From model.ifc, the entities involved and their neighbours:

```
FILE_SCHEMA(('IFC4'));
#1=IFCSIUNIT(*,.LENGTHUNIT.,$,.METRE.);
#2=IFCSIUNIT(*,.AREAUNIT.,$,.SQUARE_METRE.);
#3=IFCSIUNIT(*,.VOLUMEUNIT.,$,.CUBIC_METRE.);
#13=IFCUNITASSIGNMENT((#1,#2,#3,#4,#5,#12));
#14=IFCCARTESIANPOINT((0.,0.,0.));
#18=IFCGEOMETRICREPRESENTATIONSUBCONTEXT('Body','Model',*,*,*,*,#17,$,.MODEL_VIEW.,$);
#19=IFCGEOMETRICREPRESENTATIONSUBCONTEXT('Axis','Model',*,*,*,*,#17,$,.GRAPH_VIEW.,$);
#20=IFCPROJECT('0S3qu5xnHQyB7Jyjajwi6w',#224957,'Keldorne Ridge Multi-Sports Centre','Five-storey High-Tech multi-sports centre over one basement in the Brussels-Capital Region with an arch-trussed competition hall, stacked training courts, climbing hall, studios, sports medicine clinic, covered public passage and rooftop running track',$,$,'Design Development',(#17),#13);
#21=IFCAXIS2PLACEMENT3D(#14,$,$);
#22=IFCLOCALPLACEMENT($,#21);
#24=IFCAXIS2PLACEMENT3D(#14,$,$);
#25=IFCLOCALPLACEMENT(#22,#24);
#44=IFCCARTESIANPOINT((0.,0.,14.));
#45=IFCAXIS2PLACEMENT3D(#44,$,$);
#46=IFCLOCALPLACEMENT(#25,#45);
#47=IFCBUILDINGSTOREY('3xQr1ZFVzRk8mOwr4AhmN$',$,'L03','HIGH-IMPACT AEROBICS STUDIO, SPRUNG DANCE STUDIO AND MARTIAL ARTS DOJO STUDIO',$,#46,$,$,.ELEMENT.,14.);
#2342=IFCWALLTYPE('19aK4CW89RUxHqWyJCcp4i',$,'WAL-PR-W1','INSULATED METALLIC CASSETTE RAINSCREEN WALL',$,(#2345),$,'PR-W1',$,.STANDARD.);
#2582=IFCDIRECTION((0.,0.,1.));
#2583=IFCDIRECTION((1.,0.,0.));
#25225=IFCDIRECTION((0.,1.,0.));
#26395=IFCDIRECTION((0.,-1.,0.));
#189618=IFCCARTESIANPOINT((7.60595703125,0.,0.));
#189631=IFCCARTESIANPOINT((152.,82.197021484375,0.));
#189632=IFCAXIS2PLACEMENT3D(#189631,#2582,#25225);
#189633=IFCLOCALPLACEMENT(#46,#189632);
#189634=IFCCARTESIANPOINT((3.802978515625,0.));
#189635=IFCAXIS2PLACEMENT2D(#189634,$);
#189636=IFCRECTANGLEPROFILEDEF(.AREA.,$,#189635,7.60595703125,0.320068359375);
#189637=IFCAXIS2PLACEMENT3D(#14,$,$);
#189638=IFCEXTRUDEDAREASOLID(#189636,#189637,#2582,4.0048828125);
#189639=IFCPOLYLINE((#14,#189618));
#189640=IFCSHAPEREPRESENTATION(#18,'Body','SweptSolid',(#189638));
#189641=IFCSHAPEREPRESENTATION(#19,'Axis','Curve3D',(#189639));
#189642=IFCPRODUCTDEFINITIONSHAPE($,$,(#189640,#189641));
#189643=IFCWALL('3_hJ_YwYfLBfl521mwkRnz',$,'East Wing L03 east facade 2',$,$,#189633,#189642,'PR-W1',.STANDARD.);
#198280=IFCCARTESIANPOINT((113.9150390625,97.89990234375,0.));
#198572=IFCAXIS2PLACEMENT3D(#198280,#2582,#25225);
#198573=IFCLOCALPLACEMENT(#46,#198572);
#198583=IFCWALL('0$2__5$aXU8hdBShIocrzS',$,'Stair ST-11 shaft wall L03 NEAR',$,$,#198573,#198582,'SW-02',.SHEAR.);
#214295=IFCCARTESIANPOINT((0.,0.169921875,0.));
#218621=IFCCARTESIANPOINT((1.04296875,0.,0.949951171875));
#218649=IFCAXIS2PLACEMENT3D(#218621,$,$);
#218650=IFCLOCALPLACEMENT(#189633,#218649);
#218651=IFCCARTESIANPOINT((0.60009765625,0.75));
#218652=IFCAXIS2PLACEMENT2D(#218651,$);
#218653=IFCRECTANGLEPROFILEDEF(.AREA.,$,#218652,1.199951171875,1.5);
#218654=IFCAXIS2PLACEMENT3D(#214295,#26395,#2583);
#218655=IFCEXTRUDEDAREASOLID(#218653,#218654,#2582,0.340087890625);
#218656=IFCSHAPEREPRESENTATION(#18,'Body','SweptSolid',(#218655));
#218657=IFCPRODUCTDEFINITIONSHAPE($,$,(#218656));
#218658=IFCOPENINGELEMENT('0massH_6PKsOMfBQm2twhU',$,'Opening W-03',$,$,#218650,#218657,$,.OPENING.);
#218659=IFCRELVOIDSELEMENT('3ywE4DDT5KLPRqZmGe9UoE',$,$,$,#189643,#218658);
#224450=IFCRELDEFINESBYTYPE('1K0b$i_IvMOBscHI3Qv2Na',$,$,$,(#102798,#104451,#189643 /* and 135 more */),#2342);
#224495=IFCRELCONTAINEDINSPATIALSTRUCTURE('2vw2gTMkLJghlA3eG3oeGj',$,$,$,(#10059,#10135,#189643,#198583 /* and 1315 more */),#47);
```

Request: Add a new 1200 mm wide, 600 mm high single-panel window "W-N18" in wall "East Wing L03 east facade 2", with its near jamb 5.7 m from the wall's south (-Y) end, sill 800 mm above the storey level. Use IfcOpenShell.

```python
import numpy as np
import ifcopenshell
import ifcopenshell.api.feature
import ifcopenshell.api.geometry
import ifcopenshell.api.root
import ifcopenshell.api.spatial
import ifcopenshell.geom
import ifcopenshell.util.element
import ifcopenshell.util.placement
import ifcopenshell.util.representation
import ifcopenshell.util.shape
import ifcopenshell.util.unit

model = ifcopenshell.open("model.ifc")
unit_scale = ifcopenshell.util.unit.calculate_unit_scale(model)
settings = ifcopenshell.geom.settings()


def volume(element):
    """Net volume in cubic metres, openings subtracted."""
    shape = ifcopenshell.geom.create_shape(settings, element)
    return ifcopenshell.util.shape.get_volume(shape.geometry)


wall = model.by_guid("3_hJ_YwYfLBfl521mwkRnz")
storey = ifcopenshell.util.element.get_container(wall, ifc_class="IfcBuildingStorey")
context = ifcopenshell.util.representation.get_context(model, "Model", "Body", "MODEL_VIEW")
before = volume(wall)

width, height, from_end, sill = 1.2, 0.6, 5.7, 0.8  # metres

# The wall runs along its own X axis, and the end named is its -X end.
wall_shape = ifcopenshell.geom.create_shape(settings, wall)
x, y, z = ifcopenshell.util.shape.get_vertices(wall_shape.geometry).T
start = x.min() + from_end
face, thickness = float(y.min()), float(y.max() - y.min())
wall_matrix = ifcopenshell.util.placement.get_local_placement(wall.ObjectPlacement)
level = ifcopenshell.util.placement.get_local_placement(storey.ObjectPlacement)[2, 3]


def in_wall(x, y):
    """Placement at x, y metres in the wall's axes, at sill height."""
    matrix = wall_matrix.copy()
    matrix[:, 3] = wall_matrix @ np.array([x / unit_scale, y / unit_scale, 0.0, 1.0])
    matrix[2, 3] = level + sill / unit_scale
    return matrix


# Opening: a box that overshoots both wall faces by 50 mm.
opening = ifcopenshell.api.root.create_entity(model, ifc_class="IfcOpeningElement", predefined_type="OPENING")
box = ifcopenshell.api.geometry.add_wall_representation(
    model, context=context, length=width, height=height, thickness=thickness + 0.1
)
ifcopenshell.api.geometry.assign_representation(model, product=opening, representation=box)
ifcopenshell.api.geometry.edit_object_placement(model, product=opening, matrix=in_wall(start, face - 0.05), is_si=False)
ifcopenshell.api.feature.add_feature(model, feature=opening, element=wall)

window = ifcopenshell.api.root.create_entity(model, ifc_class="IfcWindow", name="W-N18", predefined_type="WINDOW")
window.OverallWidth, window.OverallHeight = width / unit_scale, height / unit_scale
window.PartitioningType = "SINGLE_PANEL"
body = ifcopenshell.api.geometry.add_window_representation(
    model,
    context=context,
    overall_width=window.OverallWidth,
    overall_height=window.OverallHeight,
    partition_type="SINGLE_PANEL",
)
ifcopenshell.api.geometry.assign_representation(model, product=window, representation=body)
ifcopenshell.api.spatial.assign_container(model, products=[window], relating_structure=storey)
ifcopenshell.api.feature.add_filling(model, opening=opening, element=window)

# Centre the window in the wall's thickness.
ifcopenshell.api.geometry.edit_object_placement(model, product=window, matrix=in_wall(start, face), is_si=False)
window_shape = ifcopenshell.geom.create_shape(settings, window)
depth = ifcopenshell.util.shape.get_vertices(window_shape.geometry)[:, 1]
offset = face + thickness / 2 - (depth.min() + depth.max()) / 2
ifcopenshell.api.geometry.edit_object_placement(model, product=window, matrix=in_wall(start, offset), is_si=False)

after = volume(wall)

print(f"wall volume {before:.3f} -> {after:.3f} m3")

model.write("model_rev.ifc")
```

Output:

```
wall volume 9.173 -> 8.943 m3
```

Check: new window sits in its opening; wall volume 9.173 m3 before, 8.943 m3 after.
